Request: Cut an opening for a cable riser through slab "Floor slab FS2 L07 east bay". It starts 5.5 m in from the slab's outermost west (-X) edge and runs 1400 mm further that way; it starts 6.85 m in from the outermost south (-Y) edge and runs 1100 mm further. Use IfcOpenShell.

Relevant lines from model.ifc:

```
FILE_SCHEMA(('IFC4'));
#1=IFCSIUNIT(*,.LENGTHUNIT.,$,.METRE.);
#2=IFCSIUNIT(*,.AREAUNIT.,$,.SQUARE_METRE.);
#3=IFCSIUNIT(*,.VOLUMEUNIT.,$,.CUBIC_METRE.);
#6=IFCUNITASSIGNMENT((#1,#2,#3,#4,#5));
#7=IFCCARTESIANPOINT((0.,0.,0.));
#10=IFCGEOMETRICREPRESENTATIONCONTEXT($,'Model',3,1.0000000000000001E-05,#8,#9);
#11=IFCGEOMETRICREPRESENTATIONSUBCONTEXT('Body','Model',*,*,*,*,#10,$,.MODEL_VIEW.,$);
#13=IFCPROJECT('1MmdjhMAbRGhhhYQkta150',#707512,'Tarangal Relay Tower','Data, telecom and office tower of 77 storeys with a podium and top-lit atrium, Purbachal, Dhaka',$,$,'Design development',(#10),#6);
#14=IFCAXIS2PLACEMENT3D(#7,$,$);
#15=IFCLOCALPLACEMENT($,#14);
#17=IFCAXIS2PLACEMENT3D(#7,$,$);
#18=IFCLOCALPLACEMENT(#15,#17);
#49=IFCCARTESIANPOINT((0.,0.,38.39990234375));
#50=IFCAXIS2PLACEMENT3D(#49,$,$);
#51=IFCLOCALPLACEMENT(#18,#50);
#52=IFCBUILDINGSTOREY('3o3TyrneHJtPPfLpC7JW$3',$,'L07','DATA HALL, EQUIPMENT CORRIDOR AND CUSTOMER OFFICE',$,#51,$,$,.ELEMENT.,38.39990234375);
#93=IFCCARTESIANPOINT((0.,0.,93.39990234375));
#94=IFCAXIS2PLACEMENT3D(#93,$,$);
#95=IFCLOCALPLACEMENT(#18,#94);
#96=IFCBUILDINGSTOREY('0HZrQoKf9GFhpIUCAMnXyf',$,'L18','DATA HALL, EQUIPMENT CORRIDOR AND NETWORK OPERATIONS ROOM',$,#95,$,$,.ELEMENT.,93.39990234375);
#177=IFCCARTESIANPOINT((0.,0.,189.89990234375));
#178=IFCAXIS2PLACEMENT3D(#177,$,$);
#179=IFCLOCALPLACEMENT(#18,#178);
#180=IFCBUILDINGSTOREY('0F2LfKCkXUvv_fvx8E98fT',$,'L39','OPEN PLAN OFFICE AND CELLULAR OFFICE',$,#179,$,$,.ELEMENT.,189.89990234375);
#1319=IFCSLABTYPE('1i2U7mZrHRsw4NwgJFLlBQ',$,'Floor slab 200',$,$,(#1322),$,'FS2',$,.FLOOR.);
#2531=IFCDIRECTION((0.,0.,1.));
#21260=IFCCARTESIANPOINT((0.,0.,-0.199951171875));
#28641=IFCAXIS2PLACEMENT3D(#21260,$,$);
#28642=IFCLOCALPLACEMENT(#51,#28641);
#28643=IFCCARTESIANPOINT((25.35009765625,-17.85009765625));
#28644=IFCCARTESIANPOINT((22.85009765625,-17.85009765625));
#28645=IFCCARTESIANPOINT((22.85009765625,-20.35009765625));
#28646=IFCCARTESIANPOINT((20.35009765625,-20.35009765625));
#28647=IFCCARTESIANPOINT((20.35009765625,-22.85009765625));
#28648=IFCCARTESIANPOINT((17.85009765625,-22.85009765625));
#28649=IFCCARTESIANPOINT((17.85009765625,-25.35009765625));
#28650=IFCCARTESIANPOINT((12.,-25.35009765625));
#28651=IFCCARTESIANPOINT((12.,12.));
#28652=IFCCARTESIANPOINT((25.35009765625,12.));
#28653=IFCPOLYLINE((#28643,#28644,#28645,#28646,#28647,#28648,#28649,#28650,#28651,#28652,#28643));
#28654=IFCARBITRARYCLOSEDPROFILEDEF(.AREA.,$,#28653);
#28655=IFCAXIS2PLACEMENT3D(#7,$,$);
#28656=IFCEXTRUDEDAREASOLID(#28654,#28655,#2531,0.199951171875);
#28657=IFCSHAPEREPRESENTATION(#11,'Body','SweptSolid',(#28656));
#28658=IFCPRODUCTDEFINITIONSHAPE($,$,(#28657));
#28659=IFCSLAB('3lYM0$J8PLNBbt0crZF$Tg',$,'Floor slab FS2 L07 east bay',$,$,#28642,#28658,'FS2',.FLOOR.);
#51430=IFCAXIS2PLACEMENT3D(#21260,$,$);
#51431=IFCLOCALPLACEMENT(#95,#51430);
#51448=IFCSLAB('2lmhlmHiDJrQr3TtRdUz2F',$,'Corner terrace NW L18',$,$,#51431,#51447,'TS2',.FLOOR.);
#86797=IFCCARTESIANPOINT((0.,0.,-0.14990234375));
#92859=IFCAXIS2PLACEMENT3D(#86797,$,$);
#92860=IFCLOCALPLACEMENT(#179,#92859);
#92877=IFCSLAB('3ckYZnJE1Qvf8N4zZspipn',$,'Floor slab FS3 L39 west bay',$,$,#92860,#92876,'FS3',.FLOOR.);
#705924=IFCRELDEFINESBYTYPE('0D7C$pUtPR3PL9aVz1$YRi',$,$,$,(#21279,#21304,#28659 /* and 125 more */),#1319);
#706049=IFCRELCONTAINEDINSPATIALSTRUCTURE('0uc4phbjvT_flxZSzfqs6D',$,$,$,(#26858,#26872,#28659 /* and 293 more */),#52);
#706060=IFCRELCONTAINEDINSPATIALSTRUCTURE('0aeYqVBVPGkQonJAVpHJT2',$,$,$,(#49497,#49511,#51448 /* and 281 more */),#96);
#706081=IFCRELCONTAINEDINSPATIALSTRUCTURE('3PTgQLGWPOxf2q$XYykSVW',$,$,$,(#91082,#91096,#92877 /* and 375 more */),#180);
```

```python
import numpy as np
import ifcopenshell
import ifcopenshell.api.feature
import ifcopenshell.api.geometry
import ifcopenshell.api.root
import ifcopenshell.geom
import ifcopenshell.util.placement
import ifcopenshell.util.representation
import ifcopenshell.util.shape
import ifcopenshell.util.unit

model = ifcopenshell.open("model.ifc")
unit_scale = ifcopenshell.util.unit.calculate_unit_scale(model)
settings = ifcopenshell.geom.settings()


def volume(element):
    """Net volume in cubic metres, openings subtracted."""
    shape = ifcopenshell.geom.create_shape(settings, element)
    return ifcopenshell.util.shape.get_volume(shape.geometry)


slab = model.by_guid("3lYM0$J8PLNBbt0crZF$Tg")
before = volume(slab)

# Extent in the slab's own axes, in metres. The edges named are its -X and -Y sides.
slab_shape = ifcopenshell.geom.create_shape(settings, slab)
vertices = ifcopenshell.util.shape.get_vertices(slab_shape.geometry)
x_min, y_min, bottom = vertices.min(axis=0)
top = vertices[:, 2].max()

opening = ifcopenshell.api.root.create_entity(model, ifc_class="IfcOpeningElement", name="Cable riser opening", predefined_type="OPENING")
context = ifcopenshell.util.representation.get_context(model, "Model", "Body", "MODEL_VIEW")
width, depth = 1.4, 1.1
outline = [(0.0, 0.0), (width, 0.0), (width, depth), (0.0, depth), (0.0, 0.0)]
# Overshoot both faces by 50 mm so the cut is clean.
shape = ifcopenshell.api.geometry.add_slab_representation(
    model, context=context, depth=top - bottom + 0.1, polyline=outline
)
ifcopenshell.api.geometry.assign_representation(model, product=opening, representation=shape)

matrix = ifcopenshell.util.placement.get_local_placement(slab.ObjectPlacement)
matrix[:, 3] = matrix @ np.append(np.array([x_min + 5.5, y_min + 6.85, bottom - 0.05]) / unit_scale, 1.0)
ifcopenshell.api.geometry.edit_object_placement(model, product=opening, matrix=matrix, is_si=False)
ifcopenshell.api.feature.add_feature(model, feature=opening, element=slab)

after = volume(slab)

print(f"slab volume {before:.3f} -> {after:.3f} m3")

model.write("model_rev.ifc")
```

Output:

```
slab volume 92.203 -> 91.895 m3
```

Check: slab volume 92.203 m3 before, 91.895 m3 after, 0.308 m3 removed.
